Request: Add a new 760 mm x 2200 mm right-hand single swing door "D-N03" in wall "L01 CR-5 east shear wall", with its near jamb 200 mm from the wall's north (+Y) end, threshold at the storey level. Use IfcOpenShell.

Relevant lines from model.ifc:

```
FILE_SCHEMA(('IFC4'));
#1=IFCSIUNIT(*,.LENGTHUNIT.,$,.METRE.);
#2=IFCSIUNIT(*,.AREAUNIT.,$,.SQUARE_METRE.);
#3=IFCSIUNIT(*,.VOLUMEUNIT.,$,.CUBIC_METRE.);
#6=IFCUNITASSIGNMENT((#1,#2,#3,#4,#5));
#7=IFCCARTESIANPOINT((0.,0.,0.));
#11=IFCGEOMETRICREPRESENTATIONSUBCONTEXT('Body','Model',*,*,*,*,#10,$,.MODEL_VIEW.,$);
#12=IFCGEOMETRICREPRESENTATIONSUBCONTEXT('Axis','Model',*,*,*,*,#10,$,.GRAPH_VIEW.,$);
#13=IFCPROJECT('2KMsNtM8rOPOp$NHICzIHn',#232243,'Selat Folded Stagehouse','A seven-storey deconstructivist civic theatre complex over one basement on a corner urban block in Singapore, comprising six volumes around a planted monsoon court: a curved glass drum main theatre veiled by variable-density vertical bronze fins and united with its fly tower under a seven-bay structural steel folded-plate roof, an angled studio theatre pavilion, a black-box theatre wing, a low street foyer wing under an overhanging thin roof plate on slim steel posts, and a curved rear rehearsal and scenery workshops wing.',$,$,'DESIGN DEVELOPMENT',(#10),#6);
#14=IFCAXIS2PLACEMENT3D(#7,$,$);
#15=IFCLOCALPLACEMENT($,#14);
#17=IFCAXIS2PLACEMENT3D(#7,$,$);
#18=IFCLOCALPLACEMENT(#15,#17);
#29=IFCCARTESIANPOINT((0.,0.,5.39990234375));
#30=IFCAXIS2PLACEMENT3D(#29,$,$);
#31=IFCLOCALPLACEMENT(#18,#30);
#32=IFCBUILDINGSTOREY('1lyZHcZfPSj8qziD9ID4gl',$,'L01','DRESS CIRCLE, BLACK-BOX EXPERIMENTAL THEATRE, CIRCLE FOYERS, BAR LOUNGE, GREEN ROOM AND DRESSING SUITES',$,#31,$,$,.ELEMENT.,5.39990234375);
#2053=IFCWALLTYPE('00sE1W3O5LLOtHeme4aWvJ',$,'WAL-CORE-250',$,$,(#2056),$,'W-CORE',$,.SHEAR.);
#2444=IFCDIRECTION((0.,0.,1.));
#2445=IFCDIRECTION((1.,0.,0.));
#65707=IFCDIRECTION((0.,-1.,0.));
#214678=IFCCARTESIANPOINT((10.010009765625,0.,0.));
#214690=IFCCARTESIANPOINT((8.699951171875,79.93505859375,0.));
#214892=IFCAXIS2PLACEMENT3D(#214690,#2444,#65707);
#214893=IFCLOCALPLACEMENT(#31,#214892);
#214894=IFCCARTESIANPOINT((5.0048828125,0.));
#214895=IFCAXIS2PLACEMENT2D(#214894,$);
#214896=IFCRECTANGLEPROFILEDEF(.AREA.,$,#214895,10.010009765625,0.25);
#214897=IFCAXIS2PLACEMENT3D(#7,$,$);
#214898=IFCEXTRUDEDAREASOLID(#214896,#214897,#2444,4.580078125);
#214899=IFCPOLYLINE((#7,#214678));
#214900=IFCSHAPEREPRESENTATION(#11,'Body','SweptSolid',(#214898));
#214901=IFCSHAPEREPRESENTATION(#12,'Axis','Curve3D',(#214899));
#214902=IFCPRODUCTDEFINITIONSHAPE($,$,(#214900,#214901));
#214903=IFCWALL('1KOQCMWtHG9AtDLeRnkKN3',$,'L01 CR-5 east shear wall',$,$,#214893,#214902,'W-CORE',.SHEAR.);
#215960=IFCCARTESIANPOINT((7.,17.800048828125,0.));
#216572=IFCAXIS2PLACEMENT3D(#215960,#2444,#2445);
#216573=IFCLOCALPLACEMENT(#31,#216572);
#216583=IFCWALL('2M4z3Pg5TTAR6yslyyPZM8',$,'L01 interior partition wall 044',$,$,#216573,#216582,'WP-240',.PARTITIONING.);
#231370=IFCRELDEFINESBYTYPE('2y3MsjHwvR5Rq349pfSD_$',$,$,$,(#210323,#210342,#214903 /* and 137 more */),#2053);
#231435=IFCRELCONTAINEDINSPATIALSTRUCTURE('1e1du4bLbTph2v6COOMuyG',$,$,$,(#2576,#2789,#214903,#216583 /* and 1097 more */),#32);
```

```python
import numpy as np
import ifcopenshell
import ifcopenshell.api.feature
import ifcopenshell.api.geometry
import ifcopenshell.api.root
import ifcopenshell.api.spatial
import ifcopenshell.geom
import ifcopenshell.util.element
import ifcopenshell.util.placement
import ifcopenshell.util.representation
import ifcopenshell.util.shape
import ifcopenshell.util.unit

model = ifcopenshell.open("model.ifc")
unit_scale = ifcopenshell.util.unit.calculate_unit_scale(model)
settings = ifcopenshell.geom.settings()


def volume(element):
    """Net volume in cubic metres, openings subtracted."""
    shape = ifcopenshell.geom.create_shape(settings, element)
    return ifcopenshell.util.shape.get_volume(shape.geometry)


wall = model.by_guid("1KOQCMWtHG9AtDLeRnkKN3")
storey = ifcopenshell.util.element.get_container(wall, ifc_class="IfcBuildingStorey")
context = ifcopenshell.util.representation.get_context(model, "Model", "Body", "MODEL_VIEW")
before = volume(wall)

width, height, from_end, sill = 0.76, 2.2, 0.2, 0.0  # metres

# The wall runs along its own X axis, and the end named is its -X end.
wall_shape = ifcopenshell.geom.create_shape(settings, wall)
x, y, z = ifcopenshell.util.shape.get_vertices(wall_shape.geometry).T
start = x.min() + from_end
face, thickness = float(y.min()), float(y.max() - y.min())
wall_matrix = ifcopenshell.util.placement.get_local_placement(wall.ObjectPlacement)
level = ifcopenshell.util.placement.get_local_placement(storey.ObjectPlacement)[2, 3]


def in_wall(x, y):
    """Placement at x, y metres in the wall's axes, at sill height."""
    matrix = wall_matrix.copy()
    matrix[:, 3] = wall_matrix @ np.array([x / unit_scale, y / unit_scale, 0.0, 1.0])
    matrix[2, 3] = level + sill / unit_scale
    return matrix


# Opening: a box that overshoots both wall faces by 50 mm.
opening = ifcopenshell.api.root.create_entity(model, ifc_class="IfcOpeningElement", predefined_type="OPENING")
box = ifcopenshell.api.geometry.add_wall_representation(
    model, context=context, length=width, height=height, thickness=thickness + 0.1
)
ifcopenshell.api.geometry.assign_representation(model, product=opening, representation=box)
ifcopenshell.api.geometry.edit_object_placement(model, product=opening, matrix=in_wall(start, face - 0.05), is_si=False)
ifcopenshell.api.feature.add_feature(model, feature=opening, element=wall)

door = ifcopenshell.api.root.create_entity(model, ifc_class="IfcDoor", name="D-N03", predefined_type="DOOR")
door.OverallWidth, door.OverallHeight = width / unit_scale, height / unit_scale
door.OperationType = "SINGLE_SWING_RIGHT"
body = ifcopenshell.api.geometry.add_door_representation(
    model,
    context=context,
    overall_width=door.OverallWidth,
    overall_height=door.OverallHeight,
    operation_type="SINGLE_SWING_RIGHT",
    lining_properties={"LiningDepth": thickness / unit_scale, "ThresholdDepth": thickness / unit_scale},
)
ifcopenshell.api.geometry.assign_representation(model, product=door, representation=body)
ifcopenshell.api.spatial.assign_container(model, products=[door], relating_structure=storey)
ifcopenshell.api.feature.add_filling(model, opening=opening, element=door)

# The lining spans the wall, so the door starts at the wall face.
ifcopenshell.api.geometry.edit_object_placement(model, product=door, matrix=in_wall(start, face), is_si=False)

after = volume(wall)

print(f"wall volume {before:.3f} -> {after:.3f} m3")

model.write("model_rev.ifc")
```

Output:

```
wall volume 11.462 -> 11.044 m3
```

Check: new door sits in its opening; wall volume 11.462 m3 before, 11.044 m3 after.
